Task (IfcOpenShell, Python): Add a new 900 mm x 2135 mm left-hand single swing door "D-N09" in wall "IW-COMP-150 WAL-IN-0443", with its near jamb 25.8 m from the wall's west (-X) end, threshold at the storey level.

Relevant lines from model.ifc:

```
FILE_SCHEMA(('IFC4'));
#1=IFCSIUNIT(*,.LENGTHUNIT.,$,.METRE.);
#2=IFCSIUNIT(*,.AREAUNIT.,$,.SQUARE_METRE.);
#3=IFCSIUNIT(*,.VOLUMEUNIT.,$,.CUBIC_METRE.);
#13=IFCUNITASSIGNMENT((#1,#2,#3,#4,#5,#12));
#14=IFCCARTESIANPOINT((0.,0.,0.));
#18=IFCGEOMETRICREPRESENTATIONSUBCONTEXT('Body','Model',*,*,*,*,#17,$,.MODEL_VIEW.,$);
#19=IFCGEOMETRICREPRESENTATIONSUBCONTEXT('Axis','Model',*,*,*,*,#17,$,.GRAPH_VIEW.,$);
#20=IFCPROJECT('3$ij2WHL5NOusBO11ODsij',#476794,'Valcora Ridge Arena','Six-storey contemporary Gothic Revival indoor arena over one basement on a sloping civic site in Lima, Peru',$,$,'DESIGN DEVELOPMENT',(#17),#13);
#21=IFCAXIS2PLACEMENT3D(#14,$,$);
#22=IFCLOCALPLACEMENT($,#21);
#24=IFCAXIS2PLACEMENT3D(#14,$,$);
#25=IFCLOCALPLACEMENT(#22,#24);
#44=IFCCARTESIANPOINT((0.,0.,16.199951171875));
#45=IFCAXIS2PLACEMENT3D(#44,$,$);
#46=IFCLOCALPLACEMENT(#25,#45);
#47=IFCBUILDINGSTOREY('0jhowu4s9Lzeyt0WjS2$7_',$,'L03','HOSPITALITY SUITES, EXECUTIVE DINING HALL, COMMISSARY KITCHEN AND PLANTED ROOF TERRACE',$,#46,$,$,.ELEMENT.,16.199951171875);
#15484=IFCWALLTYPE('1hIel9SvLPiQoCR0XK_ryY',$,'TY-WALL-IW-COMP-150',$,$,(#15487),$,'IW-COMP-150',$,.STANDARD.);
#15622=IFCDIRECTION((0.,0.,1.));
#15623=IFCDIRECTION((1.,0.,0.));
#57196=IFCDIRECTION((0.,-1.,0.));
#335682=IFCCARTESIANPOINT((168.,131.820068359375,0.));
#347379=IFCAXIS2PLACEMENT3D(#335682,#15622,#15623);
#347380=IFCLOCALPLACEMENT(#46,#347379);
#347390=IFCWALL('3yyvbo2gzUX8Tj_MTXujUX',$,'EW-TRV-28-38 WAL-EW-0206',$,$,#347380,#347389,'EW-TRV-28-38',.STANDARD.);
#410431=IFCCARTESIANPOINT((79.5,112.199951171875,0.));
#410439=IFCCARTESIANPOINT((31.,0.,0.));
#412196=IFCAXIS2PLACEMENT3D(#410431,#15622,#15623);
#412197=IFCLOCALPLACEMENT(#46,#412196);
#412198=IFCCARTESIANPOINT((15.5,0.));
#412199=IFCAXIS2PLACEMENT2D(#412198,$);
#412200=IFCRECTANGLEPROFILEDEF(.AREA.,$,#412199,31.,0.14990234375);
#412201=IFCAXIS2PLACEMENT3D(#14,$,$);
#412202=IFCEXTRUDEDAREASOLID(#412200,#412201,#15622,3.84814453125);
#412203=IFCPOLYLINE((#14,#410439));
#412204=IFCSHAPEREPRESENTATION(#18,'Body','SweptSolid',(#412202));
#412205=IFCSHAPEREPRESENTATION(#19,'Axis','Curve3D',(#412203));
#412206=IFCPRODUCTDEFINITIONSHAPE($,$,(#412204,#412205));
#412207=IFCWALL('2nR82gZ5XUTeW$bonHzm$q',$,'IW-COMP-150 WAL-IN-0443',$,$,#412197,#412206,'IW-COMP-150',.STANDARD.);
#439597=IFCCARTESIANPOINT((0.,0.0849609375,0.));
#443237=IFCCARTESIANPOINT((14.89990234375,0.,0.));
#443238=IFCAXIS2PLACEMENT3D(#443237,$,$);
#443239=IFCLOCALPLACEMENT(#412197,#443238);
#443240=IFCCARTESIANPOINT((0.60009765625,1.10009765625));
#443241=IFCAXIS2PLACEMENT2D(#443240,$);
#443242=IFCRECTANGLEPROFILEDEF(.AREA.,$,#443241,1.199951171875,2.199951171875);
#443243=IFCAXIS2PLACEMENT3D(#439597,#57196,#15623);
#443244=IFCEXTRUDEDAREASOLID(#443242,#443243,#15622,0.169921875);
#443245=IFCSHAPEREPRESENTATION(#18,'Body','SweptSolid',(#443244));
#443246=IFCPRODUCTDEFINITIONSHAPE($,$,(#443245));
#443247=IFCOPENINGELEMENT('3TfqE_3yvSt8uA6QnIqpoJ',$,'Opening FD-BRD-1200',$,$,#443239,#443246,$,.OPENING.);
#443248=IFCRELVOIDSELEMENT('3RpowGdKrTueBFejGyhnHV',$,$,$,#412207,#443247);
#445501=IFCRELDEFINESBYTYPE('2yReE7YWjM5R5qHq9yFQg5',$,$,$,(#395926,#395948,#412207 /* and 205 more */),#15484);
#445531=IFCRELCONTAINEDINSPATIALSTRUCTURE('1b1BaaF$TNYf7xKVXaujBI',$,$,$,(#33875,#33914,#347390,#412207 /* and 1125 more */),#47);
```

```python
import numpy as np
import ifcopenshell
import ifcopenshell.api.feature
import ifcopenshell.api.geometry
import ifcopenshell.api.root
import ifcopenshell.api.spatial
import ifcopenshell.geom
import ifcopenshell.util.element
import ifcopenshell.util.placement
import ifcopenshell.util.representation
import ifcopenshell.util.shape
import ifcopenshell.util.unit

model = ifcopenshell.open("model.ifc")
unit_scale = ifcopenshell.util.unit.calculate_unit_scale(model)
settings = ifcopenshell.geom.settings()


def volume(element):
    """Net volume in cubic metres, openings subtracted."""
    shape = ifcopenshell.geom.create_shape(settings, element)
    return ifcopenshell.util.shape.get_volume(shape.geometry)


wall = model.by_id(412207)
storey = ifcopenshell.util.element.get_container(wall, ifc_class="IfcBuildingStorey")
context = ifcopenshell.util.representation.get_context(model, "Model", "Body", "MODEL_VIEW")
before = volume(wall)

width, height, from_end, sill = 0.9, 2.135, 25.8, 0.0  # metres

# The wall runs along its own X axis, and the end named is its -X end.
wall_shape = ifcopenshell.geom.create_shape(settings, wall)
x, y, z = ifcopenshell.util.shape.get_vertices(wall_shape.geometry).T
start = x.min() + from_end
face, thickness = float(y.min()), float(y.max() - y.min())
wall_matrix = ifcopenshell.util.placement.get_local_placement(wall.ObjectPlacement)
level = ifcopenshell.util.placement.get_local_placement(storey.ObjectPlacement)[2, 3]


def in_wall(x, y):
    """Placement at x, y metres in the wall's axes, at sill height."""
    matrix = wall_matrix.copy()
    matrix[:, 3] = wall_matrix @ np.array([x / unit_scale, y / unit_scale, 0.0, 1.0])
    matrix[2, 3] = level + sill / unit_scale
    return matrix


# Opening: a box that overshoots both wall faces by 50 mm.
opening = ifcopenshell.api.root.create_entity(model, ifc_class="IfcOpeningElement", predefined_type="OPENING")
box = ifcopenshell.api.geometry.add_wall_representation(
    model, context=context, length=width, height=height, thickness=thickness + 0.1
)
ifcopenshell.api.geometry.assign_representation(model, product=opening, representation=box)
ifcopenshell.api.geometry.edit_object_placement(model, product=opening, matrix=in_wall(start, face - 0.05), is_si=False)
ifcopenshell.api.feature.add_feature(model, feature=opening, element=wall)

door = ifcopenshell.api.root.create_entity(model, ifc_class="IfcDoor", name="D-N09", predefined_type="DOOR")
door.OverallWidth, door.OverallHeight = width / unit_scale, height / unit_scale
door.OperationType = "SINGLE_SWING_LEFT"
body = ifcopenshell.api.geometry.add_door_representation(
    model,
    context=context,
    overall_width=door.OverallWidth,
    overall_height=door.OverallHeight,
    operation_type="SINGLE_SWING_LEFT",
    lining_properties={"LiningDepth": thickness / unit_scale, "ThresholdDepth": thickness / unit_scale},
)
ifcopenshell.api.geometry.assign_representation(model, product=door, representation=body)
ifcopenshell.api.spatial.assign_container(model, products=[door], relating_structure=storey)
ifcopenshell.api.feature.add_filling(model, opening=opening, element=door)

# The lining spans the wall, so the door starts at the wall face.
ifcopenshell.api.geometry.edit_object_placement(model, product=door, matrix=in_wall(start, face), is_si=False)

after = volume(wall)

print(f"wall volume {before:.3f} -> {after:.3f} m3")

model.write("model_edited.ifc")
```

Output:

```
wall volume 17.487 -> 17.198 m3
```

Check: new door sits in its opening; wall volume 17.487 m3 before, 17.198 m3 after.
